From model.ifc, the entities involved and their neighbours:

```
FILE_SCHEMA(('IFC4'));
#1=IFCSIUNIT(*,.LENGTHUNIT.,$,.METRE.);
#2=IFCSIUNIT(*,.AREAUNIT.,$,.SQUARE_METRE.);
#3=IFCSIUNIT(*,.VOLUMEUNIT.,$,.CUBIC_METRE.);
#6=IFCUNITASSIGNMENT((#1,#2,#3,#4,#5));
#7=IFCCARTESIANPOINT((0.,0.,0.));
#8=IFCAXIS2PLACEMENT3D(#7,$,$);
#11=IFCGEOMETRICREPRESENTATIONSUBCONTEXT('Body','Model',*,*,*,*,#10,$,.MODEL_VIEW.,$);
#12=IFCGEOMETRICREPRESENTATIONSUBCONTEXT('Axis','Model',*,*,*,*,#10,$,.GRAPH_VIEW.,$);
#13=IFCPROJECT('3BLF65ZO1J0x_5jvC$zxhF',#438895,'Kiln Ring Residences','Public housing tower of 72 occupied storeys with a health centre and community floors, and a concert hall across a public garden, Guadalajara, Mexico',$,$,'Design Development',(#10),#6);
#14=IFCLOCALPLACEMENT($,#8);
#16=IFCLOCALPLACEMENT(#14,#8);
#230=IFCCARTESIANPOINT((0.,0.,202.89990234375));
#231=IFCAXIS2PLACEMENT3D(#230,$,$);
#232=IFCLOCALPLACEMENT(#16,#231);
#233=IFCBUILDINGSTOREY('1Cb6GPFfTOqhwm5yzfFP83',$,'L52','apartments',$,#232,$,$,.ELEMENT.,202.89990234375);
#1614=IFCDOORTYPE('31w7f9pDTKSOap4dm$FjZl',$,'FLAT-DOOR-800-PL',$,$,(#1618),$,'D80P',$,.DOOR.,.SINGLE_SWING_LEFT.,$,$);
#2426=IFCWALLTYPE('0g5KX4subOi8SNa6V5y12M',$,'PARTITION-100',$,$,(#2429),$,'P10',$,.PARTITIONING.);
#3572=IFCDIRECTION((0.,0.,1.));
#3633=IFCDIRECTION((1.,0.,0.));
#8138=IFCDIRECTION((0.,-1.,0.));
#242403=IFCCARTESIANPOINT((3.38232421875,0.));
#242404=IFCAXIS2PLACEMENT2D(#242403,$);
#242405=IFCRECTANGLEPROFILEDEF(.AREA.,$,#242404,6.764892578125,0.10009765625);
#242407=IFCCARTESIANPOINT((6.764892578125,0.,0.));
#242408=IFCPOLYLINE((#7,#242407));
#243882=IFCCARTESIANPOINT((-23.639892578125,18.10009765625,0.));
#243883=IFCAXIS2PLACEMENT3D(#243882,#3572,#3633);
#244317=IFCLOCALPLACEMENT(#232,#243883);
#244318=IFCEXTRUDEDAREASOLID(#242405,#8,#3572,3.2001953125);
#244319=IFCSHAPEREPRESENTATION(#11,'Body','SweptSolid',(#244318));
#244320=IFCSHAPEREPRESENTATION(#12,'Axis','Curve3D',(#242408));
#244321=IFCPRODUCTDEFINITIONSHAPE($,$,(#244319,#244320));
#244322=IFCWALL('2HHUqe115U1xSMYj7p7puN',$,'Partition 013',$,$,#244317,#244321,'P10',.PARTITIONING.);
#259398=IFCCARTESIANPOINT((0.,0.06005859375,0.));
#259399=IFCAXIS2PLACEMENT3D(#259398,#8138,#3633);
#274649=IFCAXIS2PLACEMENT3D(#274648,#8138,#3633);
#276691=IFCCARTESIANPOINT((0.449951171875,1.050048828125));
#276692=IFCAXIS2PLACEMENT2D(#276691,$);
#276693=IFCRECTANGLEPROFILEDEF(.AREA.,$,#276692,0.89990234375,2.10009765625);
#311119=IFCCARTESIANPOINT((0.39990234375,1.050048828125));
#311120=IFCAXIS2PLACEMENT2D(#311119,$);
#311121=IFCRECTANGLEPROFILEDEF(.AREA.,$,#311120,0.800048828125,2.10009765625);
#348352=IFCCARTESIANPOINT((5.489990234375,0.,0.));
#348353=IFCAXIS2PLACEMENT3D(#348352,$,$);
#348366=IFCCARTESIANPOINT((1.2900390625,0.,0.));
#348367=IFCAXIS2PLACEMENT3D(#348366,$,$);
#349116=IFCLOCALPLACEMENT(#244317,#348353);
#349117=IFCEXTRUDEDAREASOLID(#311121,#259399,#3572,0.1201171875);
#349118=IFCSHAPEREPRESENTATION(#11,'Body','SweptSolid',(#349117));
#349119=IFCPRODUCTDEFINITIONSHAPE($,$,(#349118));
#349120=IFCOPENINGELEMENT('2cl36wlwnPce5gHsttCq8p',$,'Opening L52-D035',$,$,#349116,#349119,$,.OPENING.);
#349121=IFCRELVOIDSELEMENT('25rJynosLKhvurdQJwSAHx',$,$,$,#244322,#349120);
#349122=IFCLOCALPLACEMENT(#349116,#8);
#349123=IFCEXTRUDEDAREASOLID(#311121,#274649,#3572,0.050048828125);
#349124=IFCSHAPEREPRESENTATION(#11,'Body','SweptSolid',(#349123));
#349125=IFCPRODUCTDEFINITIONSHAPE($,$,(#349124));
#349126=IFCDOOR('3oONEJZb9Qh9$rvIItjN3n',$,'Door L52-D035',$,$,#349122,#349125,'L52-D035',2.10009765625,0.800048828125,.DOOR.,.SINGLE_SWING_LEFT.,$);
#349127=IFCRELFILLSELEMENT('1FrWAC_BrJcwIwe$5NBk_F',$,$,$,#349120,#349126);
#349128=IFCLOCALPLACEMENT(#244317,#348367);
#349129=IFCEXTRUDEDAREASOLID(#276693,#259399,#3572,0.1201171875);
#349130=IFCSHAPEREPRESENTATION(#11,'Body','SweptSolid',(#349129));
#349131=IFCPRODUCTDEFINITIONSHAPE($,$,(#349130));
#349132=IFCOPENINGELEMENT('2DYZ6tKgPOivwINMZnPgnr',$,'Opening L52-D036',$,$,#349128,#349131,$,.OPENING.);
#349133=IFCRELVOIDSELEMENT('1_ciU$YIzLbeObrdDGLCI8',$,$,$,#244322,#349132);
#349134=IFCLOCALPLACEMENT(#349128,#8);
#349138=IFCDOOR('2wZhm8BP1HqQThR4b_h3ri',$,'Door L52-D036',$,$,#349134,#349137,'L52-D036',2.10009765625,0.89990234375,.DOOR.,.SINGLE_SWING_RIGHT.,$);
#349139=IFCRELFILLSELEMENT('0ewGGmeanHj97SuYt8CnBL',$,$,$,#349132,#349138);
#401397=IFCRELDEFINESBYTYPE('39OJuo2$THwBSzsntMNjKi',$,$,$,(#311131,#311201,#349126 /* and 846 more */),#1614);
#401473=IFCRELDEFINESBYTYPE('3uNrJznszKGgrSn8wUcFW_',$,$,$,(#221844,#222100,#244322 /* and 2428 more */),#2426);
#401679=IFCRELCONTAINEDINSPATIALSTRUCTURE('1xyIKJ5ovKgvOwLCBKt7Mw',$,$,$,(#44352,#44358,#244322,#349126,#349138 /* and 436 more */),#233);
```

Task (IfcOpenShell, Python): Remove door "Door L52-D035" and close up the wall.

```python
import ifcopenshell
import ifcopenshell.api.feature
import ifcopenshell.api.root
import ifcopenshell.geom
import ifcopenshell.util.shape

model = ifcopenshell.open("model.ifc")
settings = ifcopenshell.geom.settings()


def volume(element):
    """Net volume in cubic metres, openings subtracted."""
    shape = ifcopenshell.geom.create_shape(settings, element)
    return ifcopenshell.util.shape.get_volume(shape.geometry)


door = model.by_id(349126)
opening = door.FillsVoids[0].RelatingOpeningElement
wall = opening.VoidsElements[0].RelatingBuildingElement
before = volume(wall)

ifcopenshell.api.root.remove_product(model, product=door)
ifcopenshell.api.feature.remove_feature(model, feature=opening)

after = volume(wall)

print(f"wall volume {before:.3f} -> {after:.3f} m3")

model.write("model_rev.ifc")
```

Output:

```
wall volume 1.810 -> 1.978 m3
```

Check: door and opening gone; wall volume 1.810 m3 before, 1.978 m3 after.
